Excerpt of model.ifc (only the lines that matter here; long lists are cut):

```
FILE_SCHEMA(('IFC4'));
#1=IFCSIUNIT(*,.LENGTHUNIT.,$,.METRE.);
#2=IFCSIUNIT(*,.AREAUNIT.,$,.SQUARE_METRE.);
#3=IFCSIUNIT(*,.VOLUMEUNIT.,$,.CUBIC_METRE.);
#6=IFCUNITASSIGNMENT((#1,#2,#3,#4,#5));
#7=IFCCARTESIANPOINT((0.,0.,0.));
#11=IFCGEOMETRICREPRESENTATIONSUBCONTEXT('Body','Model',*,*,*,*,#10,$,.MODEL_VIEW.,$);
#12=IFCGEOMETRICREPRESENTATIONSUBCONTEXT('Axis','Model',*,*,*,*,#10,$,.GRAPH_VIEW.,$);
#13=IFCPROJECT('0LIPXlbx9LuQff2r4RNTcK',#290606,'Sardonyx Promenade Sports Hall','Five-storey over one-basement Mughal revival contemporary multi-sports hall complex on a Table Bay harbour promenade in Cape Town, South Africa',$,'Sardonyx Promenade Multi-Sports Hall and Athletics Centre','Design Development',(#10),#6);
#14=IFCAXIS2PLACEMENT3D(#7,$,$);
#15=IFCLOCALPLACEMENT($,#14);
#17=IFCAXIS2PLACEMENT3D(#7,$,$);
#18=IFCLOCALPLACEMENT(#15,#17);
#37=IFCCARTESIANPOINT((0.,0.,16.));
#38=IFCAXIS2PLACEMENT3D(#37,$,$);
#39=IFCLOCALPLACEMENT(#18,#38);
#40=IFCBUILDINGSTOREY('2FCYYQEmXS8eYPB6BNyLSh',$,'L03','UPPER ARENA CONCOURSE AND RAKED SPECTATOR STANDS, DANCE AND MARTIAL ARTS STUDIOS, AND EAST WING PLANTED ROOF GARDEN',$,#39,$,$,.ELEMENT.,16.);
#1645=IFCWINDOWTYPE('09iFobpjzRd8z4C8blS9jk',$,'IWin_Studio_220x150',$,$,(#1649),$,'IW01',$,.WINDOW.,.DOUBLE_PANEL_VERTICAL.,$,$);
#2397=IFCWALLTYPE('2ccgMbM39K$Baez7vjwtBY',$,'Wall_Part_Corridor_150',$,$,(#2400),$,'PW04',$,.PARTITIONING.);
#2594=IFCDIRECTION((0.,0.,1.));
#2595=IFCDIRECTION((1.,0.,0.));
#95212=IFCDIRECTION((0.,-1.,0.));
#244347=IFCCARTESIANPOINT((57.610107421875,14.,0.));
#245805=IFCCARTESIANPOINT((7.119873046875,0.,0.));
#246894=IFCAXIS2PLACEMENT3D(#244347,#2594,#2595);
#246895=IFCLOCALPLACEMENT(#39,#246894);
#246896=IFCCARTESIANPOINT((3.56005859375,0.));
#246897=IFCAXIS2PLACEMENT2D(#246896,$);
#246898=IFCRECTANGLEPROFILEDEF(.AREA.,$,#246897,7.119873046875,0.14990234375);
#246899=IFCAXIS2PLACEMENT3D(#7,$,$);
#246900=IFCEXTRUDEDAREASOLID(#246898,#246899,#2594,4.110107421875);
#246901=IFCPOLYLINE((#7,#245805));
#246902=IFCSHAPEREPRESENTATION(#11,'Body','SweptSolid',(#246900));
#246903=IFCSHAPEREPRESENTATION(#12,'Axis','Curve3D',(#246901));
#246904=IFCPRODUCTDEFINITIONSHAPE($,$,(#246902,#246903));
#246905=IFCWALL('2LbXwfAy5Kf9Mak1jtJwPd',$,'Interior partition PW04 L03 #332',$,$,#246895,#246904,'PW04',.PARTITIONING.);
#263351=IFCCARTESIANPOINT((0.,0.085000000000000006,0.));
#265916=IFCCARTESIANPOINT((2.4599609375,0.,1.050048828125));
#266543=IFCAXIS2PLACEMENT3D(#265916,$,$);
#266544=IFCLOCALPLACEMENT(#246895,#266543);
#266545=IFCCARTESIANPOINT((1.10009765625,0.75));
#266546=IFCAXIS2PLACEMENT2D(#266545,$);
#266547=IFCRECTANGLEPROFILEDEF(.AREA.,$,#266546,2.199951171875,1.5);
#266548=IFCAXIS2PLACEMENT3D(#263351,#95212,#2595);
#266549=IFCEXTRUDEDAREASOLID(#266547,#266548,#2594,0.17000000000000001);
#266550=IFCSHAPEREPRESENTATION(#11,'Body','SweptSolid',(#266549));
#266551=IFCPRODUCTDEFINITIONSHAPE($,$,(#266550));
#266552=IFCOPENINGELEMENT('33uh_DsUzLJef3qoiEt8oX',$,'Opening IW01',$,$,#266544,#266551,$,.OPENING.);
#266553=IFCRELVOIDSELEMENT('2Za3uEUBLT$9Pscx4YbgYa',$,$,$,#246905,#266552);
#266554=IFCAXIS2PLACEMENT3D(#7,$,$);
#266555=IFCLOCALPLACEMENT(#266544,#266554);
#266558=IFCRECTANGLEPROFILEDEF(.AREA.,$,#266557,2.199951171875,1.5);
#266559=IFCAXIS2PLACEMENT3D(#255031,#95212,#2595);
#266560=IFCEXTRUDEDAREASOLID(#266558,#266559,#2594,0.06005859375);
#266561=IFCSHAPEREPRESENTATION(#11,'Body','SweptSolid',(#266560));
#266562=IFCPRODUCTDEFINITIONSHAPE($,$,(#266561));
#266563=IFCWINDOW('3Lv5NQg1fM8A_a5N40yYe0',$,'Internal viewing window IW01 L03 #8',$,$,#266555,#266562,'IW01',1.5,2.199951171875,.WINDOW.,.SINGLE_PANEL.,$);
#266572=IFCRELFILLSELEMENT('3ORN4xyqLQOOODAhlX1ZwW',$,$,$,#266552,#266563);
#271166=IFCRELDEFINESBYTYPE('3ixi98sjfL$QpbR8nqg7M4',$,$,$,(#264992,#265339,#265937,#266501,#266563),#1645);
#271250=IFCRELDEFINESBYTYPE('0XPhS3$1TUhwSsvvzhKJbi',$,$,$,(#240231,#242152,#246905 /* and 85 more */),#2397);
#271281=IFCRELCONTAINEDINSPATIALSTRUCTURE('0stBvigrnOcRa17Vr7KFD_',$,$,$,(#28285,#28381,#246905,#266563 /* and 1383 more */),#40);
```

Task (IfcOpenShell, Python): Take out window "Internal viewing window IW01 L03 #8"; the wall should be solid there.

```python
import ifcopenshell
import ifcopenshell.api.feature
import ifcopenshell.api.root
import ifcopenshell.geom
import ifcopenshell.util.shape

model = ifcopenshell.open("model.ifc")
settings = ifcopenshell.geom.settings()


def volume(element):
    """Net volume in cubic metres, openings subtracted."""
    shape = ifcopenshell.geom.create_shape(settings, element)
    return ifcopenshell.util.shape.get_volume(shape.geometry)


window = model.by_guid("3Lv5NQg1fM8A_a5N40yYe0")
opening = window.FillsVoids[0].RelatingOpeningElement
wall = opening.VoidsElements[0].RelatingBuildingElement
before = volume(wall)

ifcopenshell.api.root.remove_product(model, product=window)
ifcopenshell.api.feature.remove_feature(model, feature=opening)

after = volume(wall)

print(f"wall volume {before:.3f} -> {after:.3f} m3")

model.write("model-out.ifc")
```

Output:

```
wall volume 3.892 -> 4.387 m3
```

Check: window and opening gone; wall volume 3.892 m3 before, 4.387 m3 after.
